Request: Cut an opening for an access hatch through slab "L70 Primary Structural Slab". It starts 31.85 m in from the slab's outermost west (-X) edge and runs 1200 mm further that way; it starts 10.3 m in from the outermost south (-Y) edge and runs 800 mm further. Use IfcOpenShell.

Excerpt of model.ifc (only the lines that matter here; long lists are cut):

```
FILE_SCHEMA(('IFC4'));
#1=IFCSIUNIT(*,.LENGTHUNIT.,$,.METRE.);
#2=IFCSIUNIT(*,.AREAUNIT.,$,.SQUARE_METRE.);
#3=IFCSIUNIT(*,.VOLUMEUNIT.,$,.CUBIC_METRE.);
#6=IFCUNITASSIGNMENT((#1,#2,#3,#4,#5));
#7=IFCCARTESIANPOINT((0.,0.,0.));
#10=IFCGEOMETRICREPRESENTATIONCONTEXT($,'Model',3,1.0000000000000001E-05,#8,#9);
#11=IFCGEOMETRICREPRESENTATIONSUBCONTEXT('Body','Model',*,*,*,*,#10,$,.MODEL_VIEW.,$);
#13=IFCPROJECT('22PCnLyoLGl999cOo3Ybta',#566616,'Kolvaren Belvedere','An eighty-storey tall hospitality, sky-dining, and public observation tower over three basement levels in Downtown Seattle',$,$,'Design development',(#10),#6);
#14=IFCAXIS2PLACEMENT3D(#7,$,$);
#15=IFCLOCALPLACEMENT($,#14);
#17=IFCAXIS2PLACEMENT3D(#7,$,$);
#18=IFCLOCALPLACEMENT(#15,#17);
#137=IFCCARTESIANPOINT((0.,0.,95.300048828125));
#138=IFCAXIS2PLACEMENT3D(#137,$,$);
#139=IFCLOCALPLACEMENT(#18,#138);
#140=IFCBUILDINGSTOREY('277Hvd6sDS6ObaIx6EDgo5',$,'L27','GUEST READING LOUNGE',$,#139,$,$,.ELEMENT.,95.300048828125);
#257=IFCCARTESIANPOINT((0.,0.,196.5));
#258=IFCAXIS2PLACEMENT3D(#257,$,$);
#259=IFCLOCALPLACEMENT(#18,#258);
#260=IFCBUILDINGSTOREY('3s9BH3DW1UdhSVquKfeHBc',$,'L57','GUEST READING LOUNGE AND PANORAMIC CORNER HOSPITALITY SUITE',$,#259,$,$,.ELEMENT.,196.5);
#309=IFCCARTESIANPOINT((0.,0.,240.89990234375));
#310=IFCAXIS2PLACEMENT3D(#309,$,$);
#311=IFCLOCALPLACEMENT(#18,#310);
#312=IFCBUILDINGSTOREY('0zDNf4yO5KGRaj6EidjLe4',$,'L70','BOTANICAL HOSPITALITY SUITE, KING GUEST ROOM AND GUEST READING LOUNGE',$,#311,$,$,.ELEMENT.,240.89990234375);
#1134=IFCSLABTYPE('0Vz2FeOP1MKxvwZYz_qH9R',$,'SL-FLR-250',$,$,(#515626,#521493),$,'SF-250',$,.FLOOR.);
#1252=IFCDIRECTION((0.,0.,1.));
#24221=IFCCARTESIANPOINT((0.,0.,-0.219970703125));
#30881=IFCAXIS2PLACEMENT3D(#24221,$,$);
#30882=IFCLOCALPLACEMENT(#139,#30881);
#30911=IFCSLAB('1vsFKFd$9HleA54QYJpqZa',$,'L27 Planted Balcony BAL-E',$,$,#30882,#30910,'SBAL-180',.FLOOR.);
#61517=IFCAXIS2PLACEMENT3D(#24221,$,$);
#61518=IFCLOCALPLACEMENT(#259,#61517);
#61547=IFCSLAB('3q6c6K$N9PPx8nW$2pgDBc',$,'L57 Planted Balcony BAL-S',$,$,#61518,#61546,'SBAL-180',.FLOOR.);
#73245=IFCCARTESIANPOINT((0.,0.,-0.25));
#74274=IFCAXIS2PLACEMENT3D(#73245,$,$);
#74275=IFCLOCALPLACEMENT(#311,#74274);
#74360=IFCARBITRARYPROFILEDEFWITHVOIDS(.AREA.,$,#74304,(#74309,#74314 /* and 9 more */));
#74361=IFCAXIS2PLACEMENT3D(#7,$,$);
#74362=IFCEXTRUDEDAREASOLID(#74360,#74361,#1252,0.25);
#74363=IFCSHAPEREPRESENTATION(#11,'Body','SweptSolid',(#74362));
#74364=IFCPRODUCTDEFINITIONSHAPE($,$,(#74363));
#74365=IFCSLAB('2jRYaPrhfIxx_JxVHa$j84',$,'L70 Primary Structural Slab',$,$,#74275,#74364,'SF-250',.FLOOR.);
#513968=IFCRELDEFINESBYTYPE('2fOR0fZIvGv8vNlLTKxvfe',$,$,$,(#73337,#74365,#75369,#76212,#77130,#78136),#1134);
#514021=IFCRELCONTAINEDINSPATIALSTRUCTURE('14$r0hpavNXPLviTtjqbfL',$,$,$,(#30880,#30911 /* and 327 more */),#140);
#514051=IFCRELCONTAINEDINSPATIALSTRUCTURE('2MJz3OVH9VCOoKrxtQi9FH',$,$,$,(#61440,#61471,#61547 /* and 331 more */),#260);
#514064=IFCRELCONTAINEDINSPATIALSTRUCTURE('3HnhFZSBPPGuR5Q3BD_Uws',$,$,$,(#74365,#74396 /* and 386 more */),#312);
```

```python
import numpy as np
import ifcopenshell
import ifcopenshell.api.feature
import ifcopenshell.api.geometry
import ifcopenshell.api.root
import ifcopenshell.geom
import ifcopenshell.util.placement
import ifcopenshell.util.representation
import ifcopenshell.util.shape
import ifcopenshell.util.unit

model = ifcopenshell.open("model.ifc")
unit_scale = ifcopenshell.util.unit.calculate_unit_scale(model)
settings = ifcopenshell.geom.settings()


def volume(element):
    """Net volume in cubic metres, openings subtracted."""
    shape = ifcopenshell.geom.create_shape(settings, element)
    return ifcopenshell.util.shape.get_volume(shape.geometry)


slab = model.by_guid("2jRYaPrhfIxx_JxVHa$j84")
before = volume(slab)

# Extent in the slab's own axes, in metres. The edges named are its -X and -Y sides.
slab_shape = ifcopenshell.geom.create_shape(settings, slab)
vertices = ifcopenshell.util.shape.get_vertices(slab_shape.geometry)
x_min, y_min, bottom = vertices.min(axis=0)
top = vertices[:, 2].max()

opening = ifcopenshell.api.root.create_entity(model, ifc_class="IfcOpeningElement", name="Access hatch opening", predefined_type="OPENING")
context = ifcopenshell.util.representation.get_context(model, "Model", "Body", "MODEL_VIEW")
width, depth = 1.2, 0.8
outline = [(0.0, 0.0), (width, 0.0), (width, depth), (0.0, depth), (0.0, 0.0)]
# Overshoot both faces by 50 mm so the cut is clean.
shape = ifcopenshell.api.geometry.add_slab_representation(
    model, context=context, depth=top - bottom + 0.1, polyline=outline
)
ifcopenshell.api.geometry.assign_representation(model, product=opening, representation=shape)

matrix = ifcopenshell.util.placement.get_local_placement(slab.ObjectPlacement)
matrix[:, 3] = matrix @ np.append(np.array([x_min + 31.85, y_min + 10.3, bottom - 0.05]) / unit_scale, 1.0)
ifcopenshell.api.geometry.edit_object_placement(model, product=opening, matrix=matrix, is_si=False)
ifcopenshell.api.feature.add_feature(model, feature=opening, element=slab)

after = volume(slab)

print(f"slab volume {before:.3f} -> {after:.3f} m3")

model.write("model-out.ifc")
```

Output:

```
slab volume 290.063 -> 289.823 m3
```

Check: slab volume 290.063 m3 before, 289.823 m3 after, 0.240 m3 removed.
